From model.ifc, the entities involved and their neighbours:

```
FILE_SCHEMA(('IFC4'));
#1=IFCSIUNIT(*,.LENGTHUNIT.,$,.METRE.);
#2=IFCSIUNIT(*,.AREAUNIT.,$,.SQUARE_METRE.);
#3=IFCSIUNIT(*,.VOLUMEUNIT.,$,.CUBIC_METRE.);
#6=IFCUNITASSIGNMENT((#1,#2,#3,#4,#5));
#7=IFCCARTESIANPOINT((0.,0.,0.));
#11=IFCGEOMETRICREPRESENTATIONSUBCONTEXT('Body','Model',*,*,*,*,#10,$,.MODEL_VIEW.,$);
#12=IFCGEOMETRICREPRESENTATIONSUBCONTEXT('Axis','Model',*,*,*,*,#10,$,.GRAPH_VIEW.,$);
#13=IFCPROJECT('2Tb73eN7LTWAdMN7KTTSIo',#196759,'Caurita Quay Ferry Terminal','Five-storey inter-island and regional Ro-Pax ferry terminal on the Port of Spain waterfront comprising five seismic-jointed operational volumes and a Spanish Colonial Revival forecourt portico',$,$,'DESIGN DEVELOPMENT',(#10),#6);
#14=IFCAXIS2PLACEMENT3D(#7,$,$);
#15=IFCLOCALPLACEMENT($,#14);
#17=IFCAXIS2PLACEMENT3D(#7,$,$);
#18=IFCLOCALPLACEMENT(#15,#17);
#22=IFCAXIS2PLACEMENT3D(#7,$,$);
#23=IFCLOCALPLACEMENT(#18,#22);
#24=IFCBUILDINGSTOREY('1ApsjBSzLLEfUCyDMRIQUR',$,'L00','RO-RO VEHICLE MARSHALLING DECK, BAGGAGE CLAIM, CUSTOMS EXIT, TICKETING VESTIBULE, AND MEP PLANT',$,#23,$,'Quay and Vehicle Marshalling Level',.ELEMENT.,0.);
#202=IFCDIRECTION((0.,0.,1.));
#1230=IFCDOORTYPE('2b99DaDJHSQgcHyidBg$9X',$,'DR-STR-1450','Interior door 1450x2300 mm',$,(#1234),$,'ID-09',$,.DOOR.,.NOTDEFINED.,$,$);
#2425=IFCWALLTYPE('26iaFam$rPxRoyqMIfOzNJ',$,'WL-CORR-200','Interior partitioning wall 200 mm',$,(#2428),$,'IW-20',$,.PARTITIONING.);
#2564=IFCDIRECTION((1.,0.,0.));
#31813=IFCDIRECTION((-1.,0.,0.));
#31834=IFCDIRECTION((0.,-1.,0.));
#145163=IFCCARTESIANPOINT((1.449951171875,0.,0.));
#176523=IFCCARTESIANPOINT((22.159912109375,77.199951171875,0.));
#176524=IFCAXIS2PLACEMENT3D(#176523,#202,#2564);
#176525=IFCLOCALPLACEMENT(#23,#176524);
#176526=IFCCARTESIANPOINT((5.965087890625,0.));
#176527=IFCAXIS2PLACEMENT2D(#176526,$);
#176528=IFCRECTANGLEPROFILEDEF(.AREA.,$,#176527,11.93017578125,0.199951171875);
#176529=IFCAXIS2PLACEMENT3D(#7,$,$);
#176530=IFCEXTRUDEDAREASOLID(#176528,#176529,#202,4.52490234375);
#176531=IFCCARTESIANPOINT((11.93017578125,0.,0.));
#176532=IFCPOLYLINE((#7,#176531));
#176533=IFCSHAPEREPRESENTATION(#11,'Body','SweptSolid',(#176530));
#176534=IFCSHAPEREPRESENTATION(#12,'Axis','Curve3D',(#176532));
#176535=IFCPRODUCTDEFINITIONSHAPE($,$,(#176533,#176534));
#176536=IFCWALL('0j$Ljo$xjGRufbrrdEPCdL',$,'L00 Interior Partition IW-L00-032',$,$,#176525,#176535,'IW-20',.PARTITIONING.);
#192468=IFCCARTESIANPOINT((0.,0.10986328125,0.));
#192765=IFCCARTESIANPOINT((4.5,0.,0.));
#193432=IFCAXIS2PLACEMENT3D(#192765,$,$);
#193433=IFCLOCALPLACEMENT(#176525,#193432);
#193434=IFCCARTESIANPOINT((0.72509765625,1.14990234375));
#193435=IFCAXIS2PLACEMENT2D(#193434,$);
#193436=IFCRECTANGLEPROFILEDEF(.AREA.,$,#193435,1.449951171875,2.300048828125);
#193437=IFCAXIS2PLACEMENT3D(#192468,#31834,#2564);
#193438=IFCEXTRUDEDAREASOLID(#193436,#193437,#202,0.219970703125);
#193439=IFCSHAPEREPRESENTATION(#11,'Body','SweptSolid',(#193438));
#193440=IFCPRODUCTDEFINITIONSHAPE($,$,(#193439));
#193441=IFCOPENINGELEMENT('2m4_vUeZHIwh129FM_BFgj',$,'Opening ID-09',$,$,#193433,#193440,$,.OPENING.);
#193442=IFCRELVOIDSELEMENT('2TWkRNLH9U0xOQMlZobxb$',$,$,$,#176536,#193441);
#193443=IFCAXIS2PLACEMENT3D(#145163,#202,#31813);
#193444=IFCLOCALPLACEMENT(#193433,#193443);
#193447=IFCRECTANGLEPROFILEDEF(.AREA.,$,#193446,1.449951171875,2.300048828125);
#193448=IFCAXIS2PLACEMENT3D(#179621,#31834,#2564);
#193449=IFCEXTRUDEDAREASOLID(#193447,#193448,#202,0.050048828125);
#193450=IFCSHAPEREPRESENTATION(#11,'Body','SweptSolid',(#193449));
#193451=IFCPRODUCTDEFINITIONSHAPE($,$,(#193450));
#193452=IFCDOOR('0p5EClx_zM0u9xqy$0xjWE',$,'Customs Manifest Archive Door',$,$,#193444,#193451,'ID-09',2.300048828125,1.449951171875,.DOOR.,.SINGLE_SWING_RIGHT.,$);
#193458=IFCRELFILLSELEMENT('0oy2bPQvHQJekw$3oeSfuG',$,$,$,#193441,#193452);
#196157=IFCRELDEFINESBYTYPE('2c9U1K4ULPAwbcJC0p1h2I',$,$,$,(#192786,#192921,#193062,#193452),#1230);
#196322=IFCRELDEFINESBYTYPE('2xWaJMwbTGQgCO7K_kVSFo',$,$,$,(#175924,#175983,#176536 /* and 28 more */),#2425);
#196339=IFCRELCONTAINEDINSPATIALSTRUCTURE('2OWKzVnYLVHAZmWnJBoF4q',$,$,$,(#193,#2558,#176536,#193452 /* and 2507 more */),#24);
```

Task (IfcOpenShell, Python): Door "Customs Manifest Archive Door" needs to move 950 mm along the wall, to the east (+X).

```python
import ifcopenshell
import ifcopenshell.api.geometry
import ifcopenshell.util.placement
import ifcopenshell.util.unit

model = ifcopenshell.open("model.ifc")
unit_scale = ifcopenshell.util.unit.calculate_unit_scale(model)

door = model.by_id(193452)
opening = door.FillsVoids[0].RelatingOpeningElement
wall = opening.VoidsElements[0].RelatingBuildingElement

wall_matrix = ifcopenshell.util.placement.get_local_placement(wall.ObjectPlacement)
shift = wall_matrix[:3, 0] * 0.95 / unit_scale
before = ifcopenshell.util.placement.get_local_placement(door.ObjectPlacement)[:3, 3].copy()

# The door is placed relative to its opening, so it follows when the opening moves.
matrix = ifcopenshell.util.placement.get_local_placement(opening.ObjectPlacement)
matrix[:3, 3] += shift
ifcopenshell.api.geometry.edit_object_placement(
    model, product=opening, matrix=matrix, is_si=False, should_transform_children=True
)

after = ifcopenshell.util.placement.get_local_placement(door.ObjectPlacement)[:3, 3]
print("door moved by", (after - before).round(3) + 0.0)

model.write("model_updated.ifc")
```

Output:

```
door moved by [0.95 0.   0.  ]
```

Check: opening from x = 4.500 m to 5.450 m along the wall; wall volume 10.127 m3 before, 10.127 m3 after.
